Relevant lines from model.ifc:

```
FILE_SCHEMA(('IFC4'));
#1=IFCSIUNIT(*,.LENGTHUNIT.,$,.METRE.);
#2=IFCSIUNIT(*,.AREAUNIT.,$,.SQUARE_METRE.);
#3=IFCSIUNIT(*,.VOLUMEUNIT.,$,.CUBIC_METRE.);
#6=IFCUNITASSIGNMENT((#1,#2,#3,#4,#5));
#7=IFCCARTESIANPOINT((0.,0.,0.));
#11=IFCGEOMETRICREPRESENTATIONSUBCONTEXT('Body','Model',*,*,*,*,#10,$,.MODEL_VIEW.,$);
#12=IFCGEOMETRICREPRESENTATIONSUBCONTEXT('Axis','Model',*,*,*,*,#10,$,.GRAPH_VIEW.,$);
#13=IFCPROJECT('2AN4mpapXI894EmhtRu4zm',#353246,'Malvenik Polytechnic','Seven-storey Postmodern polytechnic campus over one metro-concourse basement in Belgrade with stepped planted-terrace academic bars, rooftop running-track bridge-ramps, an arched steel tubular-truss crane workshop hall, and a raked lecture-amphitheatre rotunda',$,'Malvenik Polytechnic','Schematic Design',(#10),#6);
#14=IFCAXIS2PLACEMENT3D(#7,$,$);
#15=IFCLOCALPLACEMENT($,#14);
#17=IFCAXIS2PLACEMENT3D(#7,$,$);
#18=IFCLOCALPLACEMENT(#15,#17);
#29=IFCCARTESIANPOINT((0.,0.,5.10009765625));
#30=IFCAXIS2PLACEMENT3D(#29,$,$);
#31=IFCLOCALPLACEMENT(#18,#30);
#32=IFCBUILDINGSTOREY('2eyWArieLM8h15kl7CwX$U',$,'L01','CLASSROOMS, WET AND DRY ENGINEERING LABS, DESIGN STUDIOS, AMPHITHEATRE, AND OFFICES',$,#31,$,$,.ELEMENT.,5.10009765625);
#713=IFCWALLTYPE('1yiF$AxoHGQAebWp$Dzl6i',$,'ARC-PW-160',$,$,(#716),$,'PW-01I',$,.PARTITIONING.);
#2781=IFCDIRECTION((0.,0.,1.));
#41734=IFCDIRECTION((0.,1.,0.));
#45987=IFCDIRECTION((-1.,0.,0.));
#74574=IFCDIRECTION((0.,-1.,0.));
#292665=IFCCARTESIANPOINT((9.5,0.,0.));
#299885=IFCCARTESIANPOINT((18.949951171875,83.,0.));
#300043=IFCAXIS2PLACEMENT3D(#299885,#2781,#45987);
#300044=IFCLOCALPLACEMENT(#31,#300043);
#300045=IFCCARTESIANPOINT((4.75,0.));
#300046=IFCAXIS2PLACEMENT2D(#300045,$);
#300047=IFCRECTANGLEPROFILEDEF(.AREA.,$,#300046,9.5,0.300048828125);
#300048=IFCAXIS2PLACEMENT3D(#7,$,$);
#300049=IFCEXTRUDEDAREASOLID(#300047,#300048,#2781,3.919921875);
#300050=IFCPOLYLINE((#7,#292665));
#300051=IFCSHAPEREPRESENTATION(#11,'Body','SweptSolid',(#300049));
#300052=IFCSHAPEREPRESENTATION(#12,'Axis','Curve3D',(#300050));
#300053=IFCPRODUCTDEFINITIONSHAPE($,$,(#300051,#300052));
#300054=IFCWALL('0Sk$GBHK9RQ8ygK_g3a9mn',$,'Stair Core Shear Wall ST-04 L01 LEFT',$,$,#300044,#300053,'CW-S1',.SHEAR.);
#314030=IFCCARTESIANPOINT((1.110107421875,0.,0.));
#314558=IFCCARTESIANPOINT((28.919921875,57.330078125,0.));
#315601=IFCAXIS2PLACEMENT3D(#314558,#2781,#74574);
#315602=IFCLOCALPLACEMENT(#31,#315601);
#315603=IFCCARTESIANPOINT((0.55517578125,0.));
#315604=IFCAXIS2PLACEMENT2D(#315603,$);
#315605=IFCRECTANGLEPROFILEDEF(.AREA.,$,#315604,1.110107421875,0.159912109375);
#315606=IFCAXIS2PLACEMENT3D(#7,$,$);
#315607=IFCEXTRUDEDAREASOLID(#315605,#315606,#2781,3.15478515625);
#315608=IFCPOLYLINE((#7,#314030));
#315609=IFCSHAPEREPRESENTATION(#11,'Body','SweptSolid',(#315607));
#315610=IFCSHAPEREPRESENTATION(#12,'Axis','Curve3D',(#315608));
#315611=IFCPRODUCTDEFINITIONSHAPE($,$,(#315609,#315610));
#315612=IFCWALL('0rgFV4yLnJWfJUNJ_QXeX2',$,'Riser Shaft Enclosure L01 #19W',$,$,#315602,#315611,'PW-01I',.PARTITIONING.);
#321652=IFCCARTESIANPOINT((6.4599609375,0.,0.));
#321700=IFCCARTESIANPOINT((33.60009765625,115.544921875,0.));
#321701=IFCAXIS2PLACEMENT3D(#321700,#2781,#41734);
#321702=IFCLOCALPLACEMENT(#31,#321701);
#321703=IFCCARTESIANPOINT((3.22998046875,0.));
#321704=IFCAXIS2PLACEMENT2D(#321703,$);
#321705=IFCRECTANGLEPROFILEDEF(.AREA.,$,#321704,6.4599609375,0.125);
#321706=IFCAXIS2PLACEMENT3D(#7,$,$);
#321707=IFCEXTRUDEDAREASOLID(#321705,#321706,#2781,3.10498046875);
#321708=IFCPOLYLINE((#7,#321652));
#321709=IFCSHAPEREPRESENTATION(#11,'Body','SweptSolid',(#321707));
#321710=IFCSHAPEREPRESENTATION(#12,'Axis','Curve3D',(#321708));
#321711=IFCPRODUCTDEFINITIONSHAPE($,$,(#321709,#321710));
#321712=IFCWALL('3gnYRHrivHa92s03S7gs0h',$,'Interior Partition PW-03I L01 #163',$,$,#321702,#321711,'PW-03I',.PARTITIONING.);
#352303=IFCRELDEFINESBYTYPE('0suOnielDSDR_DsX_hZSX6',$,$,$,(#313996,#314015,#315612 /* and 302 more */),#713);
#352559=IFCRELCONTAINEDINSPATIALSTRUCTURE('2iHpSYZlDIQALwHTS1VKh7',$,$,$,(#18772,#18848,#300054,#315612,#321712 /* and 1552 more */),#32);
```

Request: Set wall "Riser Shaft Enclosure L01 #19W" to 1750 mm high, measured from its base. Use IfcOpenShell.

```python
import ifcopenshell
import ifcopenshell.geom
import ifcopenshell.util.representation
import ifcopenshell.util.shape
import ifcopenshell.util.unit

model = ifcopenshell.open("model.ifc")
unit_scale = ifcopenshell.util.unit.calculate_unit_scale(model)
settings = ifcopenshell.geom.settings()


def volume(element):
    """Net volume in cubic metres, openings subtracted."""
    shape = ifcopenshell.geom.create_shape(settings, element)
    return ifcopenshell.util.shape.get_volume(shape.geometry)


wall = model.by_guid("0rgFV4yLnJWfJUNJ_QXeX2")
before = volume(wall)

body = ifcopenshell.util.representation.get_representation(wall, "Model", "Body")
solid = body.Items[0]
old_height = solid.Depth
solid.Depth = 1.75 / unit_scale
after = volume(wall)

print(f"height {old_height:g} -> {solid.Depth:g}, volume {before:.3f} -> {after:.3f} m3")

model.write("model_rev.ifc")
```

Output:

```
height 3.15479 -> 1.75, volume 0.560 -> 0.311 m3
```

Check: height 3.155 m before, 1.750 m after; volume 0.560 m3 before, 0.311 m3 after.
